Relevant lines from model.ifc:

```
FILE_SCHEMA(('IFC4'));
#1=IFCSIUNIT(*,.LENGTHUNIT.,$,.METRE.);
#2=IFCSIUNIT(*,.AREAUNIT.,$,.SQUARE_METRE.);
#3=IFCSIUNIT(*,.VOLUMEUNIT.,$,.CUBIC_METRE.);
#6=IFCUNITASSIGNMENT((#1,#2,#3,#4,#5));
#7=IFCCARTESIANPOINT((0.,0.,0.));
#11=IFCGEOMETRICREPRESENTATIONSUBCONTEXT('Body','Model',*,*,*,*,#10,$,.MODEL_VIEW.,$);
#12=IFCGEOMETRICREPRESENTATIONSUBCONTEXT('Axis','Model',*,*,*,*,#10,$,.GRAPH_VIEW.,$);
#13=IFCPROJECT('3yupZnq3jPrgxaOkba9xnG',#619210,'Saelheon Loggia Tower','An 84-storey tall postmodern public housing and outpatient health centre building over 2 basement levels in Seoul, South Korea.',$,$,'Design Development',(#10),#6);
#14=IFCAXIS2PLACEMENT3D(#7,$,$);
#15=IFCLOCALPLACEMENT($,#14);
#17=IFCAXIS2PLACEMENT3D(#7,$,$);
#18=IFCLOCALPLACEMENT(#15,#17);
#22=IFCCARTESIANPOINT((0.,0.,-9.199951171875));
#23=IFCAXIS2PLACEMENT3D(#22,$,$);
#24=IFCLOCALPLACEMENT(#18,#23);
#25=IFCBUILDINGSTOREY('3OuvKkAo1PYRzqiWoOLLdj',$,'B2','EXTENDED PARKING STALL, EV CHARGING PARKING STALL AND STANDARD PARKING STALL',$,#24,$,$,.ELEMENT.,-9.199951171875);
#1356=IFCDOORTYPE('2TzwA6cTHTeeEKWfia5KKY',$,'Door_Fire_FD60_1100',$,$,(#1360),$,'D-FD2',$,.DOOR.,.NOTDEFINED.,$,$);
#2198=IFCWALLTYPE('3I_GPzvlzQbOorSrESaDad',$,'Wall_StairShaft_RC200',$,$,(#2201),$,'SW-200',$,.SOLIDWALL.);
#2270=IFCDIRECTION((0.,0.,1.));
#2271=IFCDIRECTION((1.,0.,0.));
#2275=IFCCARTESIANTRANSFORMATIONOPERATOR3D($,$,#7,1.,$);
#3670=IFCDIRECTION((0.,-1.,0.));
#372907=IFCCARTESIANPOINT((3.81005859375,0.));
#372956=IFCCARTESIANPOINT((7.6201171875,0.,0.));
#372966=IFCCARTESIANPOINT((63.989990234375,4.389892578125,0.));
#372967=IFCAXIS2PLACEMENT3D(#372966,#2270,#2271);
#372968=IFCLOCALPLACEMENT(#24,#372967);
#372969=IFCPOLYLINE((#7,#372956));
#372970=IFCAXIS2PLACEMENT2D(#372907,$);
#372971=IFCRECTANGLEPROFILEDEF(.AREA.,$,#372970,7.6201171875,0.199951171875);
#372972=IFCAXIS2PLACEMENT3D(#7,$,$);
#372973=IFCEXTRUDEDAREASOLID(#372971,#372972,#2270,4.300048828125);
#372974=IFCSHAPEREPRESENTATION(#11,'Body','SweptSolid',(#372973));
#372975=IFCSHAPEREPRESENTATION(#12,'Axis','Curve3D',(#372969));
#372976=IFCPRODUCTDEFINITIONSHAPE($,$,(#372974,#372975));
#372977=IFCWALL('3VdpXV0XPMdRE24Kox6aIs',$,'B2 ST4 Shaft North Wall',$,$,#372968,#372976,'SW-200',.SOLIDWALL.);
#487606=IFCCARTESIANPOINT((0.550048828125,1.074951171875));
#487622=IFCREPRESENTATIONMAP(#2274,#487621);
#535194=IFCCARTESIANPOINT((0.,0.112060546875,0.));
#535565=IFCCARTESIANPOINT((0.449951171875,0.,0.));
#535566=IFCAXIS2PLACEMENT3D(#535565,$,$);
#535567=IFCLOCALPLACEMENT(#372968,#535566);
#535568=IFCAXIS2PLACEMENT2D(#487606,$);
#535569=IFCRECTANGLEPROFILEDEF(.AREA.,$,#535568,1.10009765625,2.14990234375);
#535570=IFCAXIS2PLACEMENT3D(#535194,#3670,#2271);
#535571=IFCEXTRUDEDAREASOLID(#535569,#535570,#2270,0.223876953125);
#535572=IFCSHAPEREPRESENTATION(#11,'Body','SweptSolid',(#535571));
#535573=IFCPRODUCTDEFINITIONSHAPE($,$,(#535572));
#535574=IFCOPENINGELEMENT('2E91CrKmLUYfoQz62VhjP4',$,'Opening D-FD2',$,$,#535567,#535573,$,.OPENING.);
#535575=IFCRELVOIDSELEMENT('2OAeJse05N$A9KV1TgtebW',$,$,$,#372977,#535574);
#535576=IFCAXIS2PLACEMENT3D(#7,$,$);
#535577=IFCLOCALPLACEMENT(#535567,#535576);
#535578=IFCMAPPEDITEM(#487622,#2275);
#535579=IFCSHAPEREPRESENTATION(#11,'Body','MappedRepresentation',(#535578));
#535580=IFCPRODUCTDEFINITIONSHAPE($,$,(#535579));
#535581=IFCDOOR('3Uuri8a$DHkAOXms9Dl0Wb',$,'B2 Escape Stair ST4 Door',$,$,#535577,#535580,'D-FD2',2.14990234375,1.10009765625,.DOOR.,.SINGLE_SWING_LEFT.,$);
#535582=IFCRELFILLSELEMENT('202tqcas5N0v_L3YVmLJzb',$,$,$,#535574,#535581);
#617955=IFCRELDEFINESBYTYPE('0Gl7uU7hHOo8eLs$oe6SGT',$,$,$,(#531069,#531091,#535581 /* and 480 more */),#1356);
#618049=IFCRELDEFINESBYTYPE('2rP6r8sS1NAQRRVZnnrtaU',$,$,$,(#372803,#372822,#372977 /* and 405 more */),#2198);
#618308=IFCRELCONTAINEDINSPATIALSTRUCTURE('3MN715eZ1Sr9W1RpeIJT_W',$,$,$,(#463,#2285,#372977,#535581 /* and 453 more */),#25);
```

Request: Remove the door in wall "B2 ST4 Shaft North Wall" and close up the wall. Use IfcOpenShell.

```python
import ifcopenshell
import ifcopenshell.api.feature
import ifcopenshell.api.root
import ifcopenshell.geom
import ifcopenshell.util.shape

model = ifcopenshell.open("model.ifc")
settings = ifcopenshell.geom.settings()


def volume(element):
    """Net volume in cubic metres, openings subtracted."""
    shape = ifcopenshell.geom.create_shape(settings, element)
    return ifcopenshell.util.shape.get_volume(shape.geometry)


door = model.by_id(535581)
opening = door.FillsVoids[0].RelatingOpeningElement
wall = opening.VoidsElements[0].RelatingBuildingElement
before = volume(wall)

ifcopenshell.api.root.remove_product(model, product=door)
ifcopenshell.api.feature.remove_feature(model, feature=opening)

after = volume(wall)

print(f"wall volume {before:.3f} -> {after:.3f} m3")

model.write("model_v2.ifc")
```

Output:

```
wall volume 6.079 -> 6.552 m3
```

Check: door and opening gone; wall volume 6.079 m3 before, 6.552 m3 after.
